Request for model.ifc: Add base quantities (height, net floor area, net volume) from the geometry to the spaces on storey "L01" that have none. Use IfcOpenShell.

First a look at what the model holds.

```python
import ifcopenshell
import ifcopenshell.util.element
import ifcopenshell.util.unit

model = ifcopenshell.open("model.ifc")
print(model.schema)
for unit_type in ("LENGTHUNIT", "AREAUNIT", "VOLUMEUNIT"):
    print(unit_type, ifcopenshell.util.unit.calculate_unit_scale(model, unit_type))
storey = next(s for s in model.by_type("IfcBuildingStorey") if s.Name == "L01")
spaces = [e for e in ifcopenshell.util.element.get_decomposition(storey) if e.is_a("IfcSpace")]
for e in sorted(spaces, key=lambda e: e.id()):
    print(e.id(), e.is_a(), e.Name, list(ifcopenshell.util.element.get_psets(e, qtos_only=True)), sep=" | ")
```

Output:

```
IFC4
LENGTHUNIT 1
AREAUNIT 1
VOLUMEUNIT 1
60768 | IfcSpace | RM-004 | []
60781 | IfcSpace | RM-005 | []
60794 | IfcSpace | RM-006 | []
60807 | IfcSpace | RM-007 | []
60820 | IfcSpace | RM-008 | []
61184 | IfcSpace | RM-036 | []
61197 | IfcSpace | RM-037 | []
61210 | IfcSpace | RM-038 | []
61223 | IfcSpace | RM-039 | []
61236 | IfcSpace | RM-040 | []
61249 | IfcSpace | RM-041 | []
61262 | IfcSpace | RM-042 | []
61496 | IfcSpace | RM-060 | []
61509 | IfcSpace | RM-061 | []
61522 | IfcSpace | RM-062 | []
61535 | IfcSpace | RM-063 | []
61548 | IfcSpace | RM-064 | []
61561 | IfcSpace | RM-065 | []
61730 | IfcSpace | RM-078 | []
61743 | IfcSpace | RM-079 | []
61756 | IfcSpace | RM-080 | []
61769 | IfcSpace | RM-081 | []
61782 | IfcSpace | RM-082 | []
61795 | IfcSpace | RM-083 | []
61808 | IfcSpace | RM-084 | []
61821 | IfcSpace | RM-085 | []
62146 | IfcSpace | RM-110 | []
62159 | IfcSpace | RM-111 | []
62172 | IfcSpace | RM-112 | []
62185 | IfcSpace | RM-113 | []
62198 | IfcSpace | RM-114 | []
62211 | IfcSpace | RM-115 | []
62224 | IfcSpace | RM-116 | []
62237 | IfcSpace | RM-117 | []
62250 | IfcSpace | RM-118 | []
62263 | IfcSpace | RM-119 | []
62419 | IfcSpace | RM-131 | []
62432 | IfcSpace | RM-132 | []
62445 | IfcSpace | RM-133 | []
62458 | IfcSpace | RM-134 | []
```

```python
import ifcopenshell
import ifcopenshell.api.pset
import ifcopenshell.geom
import ifcopenshell.util.element
import ifcopenshell.util.shape
import ifcopenshell.util.unit

model = ifcopenshell.open("model.ifc")
unit_scale = ifcopenshell.util.unit.calculate_unit_scale(model)
area_scale = ifcopenshell.util.unit.calculate_unit_scale(model, "AREAUNIT")
volume_scale = ifcopenshell.util.unit.calculate_unit_scale(model, "VOLUMEUNIT")
settings = ifcopenshell.geom.settings()

storey = next(s for s in model.by_type("IfcBuildingStorey") if s.Name == "L01")
spaces = [e for e in ifcopenshell.util.element.get_decomposition(storey) if e.is_a("IfcSpace")]

for e in sorted(spaces, key=lambda e: e.id()):
    if ifcopenshell.util.element.get_psets(e, qtos_only=True, should_inherit=False):
        continue
    # Geometry comes back in metres, in the element's own axes.
    shape = ifcopenshell.geom.create_shape(settings, e)
    values = {
        "Height": ifcopenshell.util.shape.get_z(shape.geometry) / unit_scale,
        "NetFloorArea": ifcopenshell.util.shape.get_footprint_area(shape.geometry) / area_scale,
        "NetVolume": ifcopenshell.util.shape.get_volume(shape.geometry) / volume_scale,
    }
    qto = ifcopenshell.api.pset.add_qto(model, product=e, name="Qto_SpaceBaseQuantities")
    ifcopenshell.api.pset.edit_qto(model, qto=qto, properties=values)
    print(e.id(), {k: round(v, 3) for k, v in values.items()})

model.write("model_updated.ifc")
```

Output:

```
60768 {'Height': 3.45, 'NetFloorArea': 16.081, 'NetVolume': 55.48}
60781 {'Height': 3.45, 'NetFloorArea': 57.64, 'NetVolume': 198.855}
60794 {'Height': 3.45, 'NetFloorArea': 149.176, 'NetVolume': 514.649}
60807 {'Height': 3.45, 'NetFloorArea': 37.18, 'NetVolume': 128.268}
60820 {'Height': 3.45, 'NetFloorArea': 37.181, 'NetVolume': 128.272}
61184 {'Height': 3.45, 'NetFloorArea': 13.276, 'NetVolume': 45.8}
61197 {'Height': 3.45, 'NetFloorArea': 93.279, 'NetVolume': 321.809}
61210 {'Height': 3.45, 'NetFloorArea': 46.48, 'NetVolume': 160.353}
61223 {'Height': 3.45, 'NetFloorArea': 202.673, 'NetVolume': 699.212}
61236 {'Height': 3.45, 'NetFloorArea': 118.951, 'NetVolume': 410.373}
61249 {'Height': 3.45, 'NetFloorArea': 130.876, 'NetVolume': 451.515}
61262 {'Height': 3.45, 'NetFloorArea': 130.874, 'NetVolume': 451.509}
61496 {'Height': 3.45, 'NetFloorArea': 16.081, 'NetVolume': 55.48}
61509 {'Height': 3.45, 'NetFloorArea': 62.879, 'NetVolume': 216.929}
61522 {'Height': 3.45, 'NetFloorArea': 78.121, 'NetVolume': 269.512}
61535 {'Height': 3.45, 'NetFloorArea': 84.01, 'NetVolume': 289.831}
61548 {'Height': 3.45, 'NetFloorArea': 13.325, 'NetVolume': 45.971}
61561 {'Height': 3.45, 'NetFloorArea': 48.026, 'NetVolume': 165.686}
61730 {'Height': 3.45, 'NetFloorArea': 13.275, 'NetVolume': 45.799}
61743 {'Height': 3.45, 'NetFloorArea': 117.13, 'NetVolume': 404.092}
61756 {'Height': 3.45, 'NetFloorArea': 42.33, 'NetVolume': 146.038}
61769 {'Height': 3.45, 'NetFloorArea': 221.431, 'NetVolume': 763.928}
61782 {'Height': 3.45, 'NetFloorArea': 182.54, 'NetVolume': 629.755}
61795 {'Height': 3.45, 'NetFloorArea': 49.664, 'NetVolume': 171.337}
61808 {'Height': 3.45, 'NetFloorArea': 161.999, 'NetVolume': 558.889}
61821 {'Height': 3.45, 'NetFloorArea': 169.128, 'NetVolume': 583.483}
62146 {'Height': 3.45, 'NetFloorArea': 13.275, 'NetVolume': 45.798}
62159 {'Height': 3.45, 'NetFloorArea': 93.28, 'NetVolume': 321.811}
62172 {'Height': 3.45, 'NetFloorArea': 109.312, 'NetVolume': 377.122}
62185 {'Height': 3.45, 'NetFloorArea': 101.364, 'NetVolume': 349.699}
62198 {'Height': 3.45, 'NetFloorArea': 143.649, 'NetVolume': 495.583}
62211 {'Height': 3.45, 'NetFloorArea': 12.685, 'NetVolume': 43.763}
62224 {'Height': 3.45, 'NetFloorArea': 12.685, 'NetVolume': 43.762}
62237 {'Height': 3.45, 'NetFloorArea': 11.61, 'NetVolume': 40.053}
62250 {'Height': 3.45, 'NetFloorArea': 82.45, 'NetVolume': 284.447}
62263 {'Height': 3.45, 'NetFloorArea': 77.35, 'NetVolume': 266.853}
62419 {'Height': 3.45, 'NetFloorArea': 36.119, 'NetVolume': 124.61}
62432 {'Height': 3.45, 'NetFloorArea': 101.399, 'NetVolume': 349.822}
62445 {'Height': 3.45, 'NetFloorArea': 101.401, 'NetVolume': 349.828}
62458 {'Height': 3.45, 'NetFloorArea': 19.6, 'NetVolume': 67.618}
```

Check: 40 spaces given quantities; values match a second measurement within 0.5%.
